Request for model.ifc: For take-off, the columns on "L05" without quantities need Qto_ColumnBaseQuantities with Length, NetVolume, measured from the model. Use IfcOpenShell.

First a look at what the model holds.

```python
import ifcopenshell
import ifcopenshell.util.element
import ifcopenshell.util.unit

model = ifcopenshell.open("model.ifc")
print(model.schema)
for unit_type in ("LENGTHUNIT", "AREAUNIT", "VOLUMEUNIT"):
    print(unit_type, ifcopenshell.util.unit.calculate_unit_scale(model, unit_type))
storey = next(s for s in model.by_type("IfcBuildingStorey") if s.Name == "L05")
columns = [e for e in ifcopenshell.util.element.get_decomposition(storey) if e.is_a("IfcColumn")]
for e in sorted(columns, key=lambda e: e.id()):
    print(e.id(), e.is_a(), e.Name, list(ifcopenshell.util.element.get_psets(e, qtos_only=True)), sep=" | ")
```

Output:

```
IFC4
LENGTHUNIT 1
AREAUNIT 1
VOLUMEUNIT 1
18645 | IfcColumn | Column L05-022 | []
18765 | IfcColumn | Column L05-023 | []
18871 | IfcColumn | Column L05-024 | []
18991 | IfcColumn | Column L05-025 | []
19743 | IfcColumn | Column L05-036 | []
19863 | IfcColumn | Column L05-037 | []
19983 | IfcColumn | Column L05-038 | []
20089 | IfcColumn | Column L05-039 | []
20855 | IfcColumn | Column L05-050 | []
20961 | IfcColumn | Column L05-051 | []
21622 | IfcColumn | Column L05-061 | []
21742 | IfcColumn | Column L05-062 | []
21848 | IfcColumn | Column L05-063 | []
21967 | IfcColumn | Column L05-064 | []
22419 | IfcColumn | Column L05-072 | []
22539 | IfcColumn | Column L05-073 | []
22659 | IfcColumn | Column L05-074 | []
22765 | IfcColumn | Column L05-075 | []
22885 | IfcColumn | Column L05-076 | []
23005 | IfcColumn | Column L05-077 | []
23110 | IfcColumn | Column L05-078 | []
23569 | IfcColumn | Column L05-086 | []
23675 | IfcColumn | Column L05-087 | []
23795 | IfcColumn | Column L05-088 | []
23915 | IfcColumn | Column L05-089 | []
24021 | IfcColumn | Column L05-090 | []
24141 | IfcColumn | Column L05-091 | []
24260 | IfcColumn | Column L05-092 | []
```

```python
import ifcopenshell
import ifcopenshell.api.pset
import ifcopenshell.geom
import ifcopenshell.util.element
import ifcopenshell.util.shape
import ifcopenshell.util.unit

model = ifcopenshell.open("model.ifc")
unit_scale = ifcopenshell.util.unit.calculate_unit_scale(model)
volume_scale = ifcopenshell.util.unit.calculate_unit_scale(model, "VOLUMEUNIT")
settings = ifcopenshell.geom.settings()

storey = next(s for s in model.by_type("IfcBuildingStorey") if s.Name == "L05")
columns = [e for e in ifcopenshell.util.element.get_decomposition(storey) if e.is_a("IfcColumn")]

for e in sorted(columns, key=lambda e: e.id()):
    if ifcopenshell.util.element.get_psets(e, qtos_only=True, should_inherit=False):
        continue
    # Geometry comes back in metres, in the element's own axes.
    shape = ifcopenshell.geom.create_shape(settings, e)
    values = {
        "Length": ifcopenshell.util.shape.get_z(shape.geometry) / unit_scale,
        "NetVolume": ifcopenshell.util.shape.get_volume(shape.geometry) / volume_scale,
    }
    qto = ifcopenshell.api.pset.add_qto(model, product=e, name="Qto_ColumnBaseQuantities")
    ifcopenshell.api.pset.edit_qto(model, qto=qto, properties=values)
    print(e.id(), {k: round(v, 3) for k, v in values.items()})

model.write("model_edited.ifc")
```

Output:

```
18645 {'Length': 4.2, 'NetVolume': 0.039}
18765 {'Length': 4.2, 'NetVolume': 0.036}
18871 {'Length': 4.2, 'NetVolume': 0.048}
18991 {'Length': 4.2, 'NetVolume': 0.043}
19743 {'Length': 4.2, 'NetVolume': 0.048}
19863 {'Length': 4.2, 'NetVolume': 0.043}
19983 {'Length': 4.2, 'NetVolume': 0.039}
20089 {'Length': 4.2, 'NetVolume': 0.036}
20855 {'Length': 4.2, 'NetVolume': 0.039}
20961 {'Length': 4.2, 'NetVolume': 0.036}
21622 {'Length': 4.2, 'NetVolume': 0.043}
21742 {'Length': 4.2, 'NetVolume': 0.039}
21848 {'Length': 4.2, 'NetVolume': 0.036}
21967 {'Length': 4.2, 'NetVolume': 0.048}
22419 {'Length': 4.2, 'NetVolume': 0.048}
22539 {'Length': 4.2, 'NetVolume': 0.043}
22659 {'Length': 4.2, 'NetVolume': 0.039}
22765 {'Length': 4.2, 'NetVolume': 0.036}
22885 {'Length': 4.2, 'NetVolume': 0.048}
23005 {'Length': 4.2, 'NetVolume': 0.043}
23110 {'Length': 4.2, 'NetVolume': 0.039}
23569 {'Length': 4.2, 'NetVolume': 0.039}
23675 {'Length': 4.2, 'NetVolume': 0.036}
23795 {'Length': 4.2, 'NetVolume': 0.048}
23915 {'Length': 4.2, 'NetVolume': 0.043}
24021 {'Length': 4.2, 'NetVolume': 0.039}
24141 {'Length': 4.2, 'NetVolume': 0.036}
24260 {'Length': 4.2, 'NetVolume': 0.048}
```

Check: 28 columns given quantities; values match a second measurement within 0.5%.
